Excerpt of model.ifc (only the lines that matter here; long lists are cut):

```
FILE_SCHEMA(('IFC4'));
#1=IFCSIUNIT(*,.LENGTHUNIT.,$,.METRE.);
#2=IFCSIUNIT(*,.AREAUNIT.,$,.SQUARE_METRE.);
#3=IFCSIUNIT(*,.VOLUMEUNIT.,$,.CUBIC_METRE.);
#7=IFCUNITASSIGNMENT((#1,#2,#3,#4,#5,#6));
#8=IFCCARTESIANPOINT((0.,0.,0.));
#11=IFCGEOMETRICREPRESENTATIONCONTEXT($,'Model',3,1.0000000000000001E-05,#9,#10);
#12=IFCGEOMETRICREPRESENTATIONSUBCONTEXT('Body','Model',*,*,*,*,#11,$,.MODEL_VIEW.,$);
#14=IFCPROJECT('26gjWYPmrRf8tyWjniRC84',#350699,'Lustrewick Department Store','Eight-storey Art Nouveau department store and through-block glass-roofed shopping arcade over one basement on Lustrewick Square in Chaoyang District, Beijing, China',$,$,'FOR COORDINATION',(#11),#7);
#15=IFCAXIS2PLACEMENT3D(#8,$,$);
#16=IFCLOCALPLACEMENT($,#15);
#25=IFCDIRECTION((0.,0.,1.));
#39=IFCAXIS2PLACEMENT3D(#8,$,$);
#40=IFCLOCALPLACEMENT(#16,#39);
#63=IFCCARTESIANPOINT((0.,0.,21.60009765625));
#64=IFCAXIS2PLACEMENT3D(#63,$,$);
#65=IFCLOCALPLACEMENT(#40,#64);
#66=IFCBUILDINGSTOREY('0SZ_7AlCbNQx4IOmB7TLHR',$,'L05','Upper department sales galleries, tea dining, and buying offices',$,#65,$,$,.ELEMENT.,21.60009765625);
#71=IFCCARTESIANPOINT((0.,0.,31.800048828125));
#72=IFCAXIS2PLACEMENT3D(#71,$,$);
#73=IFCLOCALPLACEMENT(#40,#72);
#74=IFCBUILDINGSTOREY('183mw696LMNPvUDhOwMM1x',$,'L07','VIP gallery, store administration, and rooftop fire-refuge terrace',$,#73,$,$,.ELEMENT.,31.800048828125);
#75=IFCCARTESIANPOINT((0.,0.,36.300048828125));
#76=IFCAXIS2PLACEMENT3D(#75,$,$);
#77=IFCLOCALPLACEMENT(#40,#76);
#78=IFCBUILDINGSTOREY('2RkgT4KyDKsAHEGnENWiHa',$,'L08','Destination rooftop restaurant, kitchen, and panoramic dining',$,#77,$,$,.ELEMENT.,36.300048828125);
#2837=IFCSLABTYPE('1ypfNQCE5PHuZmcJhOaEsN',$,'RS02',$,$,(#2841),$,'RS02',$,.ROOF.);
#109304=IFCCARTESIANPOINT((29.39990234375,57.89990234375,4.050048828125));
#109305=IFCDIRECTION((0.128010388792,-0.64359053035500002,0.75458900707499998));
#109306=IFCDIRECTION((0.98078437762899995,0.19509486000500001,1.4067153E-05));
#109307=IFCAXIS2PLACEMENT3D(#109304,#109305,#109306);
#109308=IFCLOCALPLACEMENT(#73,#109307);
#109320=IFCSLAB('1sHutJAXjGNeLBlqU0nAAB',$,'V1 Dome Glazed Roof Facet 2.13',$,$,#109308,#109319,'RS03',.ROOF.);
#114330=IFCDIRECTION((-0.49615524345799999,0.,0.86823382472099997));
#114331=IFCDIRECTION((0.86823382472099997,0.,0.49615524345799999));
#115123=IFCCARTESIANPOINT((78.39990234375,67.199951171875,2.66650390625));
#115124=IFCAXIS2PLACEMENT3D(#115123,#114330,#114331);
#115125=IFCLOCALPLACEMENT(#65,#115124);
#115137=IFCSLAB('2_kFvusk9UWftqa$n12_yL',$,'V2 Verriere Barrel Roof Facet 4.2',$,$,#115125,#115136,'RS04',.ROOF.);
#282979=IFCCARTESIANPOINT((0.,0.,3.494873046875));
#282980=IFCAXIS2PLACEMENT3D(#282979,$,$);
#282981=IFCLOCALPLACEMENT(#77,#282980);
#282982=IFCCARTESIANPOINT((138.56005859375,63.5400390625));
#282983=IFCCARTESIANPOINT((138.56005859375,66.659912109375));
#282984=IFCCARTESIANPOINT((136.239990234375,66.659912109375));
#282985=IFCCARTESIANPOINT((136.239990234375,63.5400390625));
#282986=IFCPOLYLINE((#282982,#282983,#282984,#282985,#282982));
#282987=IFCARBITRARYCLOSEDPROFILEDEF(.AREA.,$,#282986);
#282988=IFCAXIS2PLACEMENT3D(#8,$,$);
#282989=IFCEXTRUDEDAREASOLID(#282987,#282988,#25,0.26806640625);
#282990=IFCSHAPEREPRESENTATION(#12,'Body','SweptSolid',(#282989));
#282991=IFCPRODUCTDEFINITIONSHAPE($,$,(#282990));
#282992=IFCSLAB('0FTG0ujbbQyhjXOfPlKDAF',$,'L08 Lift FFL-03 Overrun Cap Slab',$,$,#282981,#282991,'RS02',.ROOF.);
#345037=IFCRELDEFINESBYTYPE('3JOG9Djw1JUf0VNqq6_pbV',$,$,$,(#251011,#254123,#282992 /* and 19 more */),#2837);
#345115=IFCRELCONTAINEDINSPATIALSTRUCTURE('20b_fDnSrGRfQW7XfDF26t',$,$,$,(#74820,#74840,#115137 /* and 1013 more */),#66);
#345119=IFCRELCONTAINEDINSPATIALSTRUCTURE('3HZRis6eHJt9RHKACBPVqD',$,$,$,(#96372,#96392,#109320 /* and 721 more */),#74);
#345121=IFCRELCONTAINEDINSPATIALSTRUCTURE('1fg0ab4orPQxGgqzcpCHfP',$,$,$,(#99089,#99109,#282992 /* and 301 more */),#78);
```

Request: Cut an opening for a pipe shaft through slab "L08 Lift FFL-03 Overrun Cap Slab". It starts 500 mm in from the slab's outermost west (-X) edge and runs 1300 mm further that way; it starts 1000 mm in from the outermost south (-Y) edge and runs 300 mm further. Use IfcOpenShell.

```python
import numpy as np
import ifcopenshell
import ifcopenshell.api.feature
import ifcopenshell.api.geometry
import ifcopenshell.api.root
import ifcopenshell.geom
import ifcopenshell.util.placement
import ifcopenshell.util.representation
import ifcopenshell.util.shape
import ifcopenshell.util.unit

model = ifcopenshell.open("model.ifc")
unit_scale = ifcopenshell.util.unit.calculate_unit_scale(model)
settings = ifcopenshell.geom.settings()


def volume(element):
    """Net volume in cubic metres, openings subtracted."""
    shape = ifcopenshell.geom.create_shape(settings, element)
    return ifcopenshell.util.shape.get_volume(shape.geometry)


slab = model.by_id(282992)
before = volume(slab)

# Extent in the slab's own axes, in metres. The edges named are its -X and -Y sides.
slab_shape = ifcopenshell.geom.create_shape(settings, slab)
vertices = ifcopenshell.util.shape.get_vertices(slab_shape.geometry)
x_min, y_min, bottom = vertices.min(axis=0)
top = vertices[:, 2].max()

opening = ifcopenshell.api.root.create_entity(model, ifc_class="IfcOpeningElement", name="Pipe shaft opening", predefined_type="OPENING")
context = ifcopenshell.util.representation.get_context(model, "Model", "Body", "MODEL_VIEW")
width, depth = 1.3, 0.3
outline = [(0.0, 0.0), (width, 0.0), (width, depth), (0.0, depth), (0.0, 0.0)]
# Overshoot both faces by 50 mm so the cut is clean.
shape = ifcopenshell.api.geometry.add_slab_representation(
    model, context=context, depth=top - bottom + 0.1, polyline=outline
)
ifcopenshell.api.geometry.assign_representation(model, product=opening, representation=shape)

matrix = ifcopenshell.util.placement.get_local_placement(slab.ObjectPlacement)
matrix[:, 3] = matrix @ np.append(np.array([x_min + 0.5, y_min + 1, bottom - 0.05]) / unit_scale, 1.0)
ifcopenshell.api.geometry.edit_object_placement(model, product=opening, matrix=matrix, is_si=False)
ifcopenshell.api.feature.add_feature(model, feature=opening, element=slab)

after = volume(slab)

print(f"slab volume {before:.3f} -> {after:.3f} m3")

model.write("model_updated.ifc")
```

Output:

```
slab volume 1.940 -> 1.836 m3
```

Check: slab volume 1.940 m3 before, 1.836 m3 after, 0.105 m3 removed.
